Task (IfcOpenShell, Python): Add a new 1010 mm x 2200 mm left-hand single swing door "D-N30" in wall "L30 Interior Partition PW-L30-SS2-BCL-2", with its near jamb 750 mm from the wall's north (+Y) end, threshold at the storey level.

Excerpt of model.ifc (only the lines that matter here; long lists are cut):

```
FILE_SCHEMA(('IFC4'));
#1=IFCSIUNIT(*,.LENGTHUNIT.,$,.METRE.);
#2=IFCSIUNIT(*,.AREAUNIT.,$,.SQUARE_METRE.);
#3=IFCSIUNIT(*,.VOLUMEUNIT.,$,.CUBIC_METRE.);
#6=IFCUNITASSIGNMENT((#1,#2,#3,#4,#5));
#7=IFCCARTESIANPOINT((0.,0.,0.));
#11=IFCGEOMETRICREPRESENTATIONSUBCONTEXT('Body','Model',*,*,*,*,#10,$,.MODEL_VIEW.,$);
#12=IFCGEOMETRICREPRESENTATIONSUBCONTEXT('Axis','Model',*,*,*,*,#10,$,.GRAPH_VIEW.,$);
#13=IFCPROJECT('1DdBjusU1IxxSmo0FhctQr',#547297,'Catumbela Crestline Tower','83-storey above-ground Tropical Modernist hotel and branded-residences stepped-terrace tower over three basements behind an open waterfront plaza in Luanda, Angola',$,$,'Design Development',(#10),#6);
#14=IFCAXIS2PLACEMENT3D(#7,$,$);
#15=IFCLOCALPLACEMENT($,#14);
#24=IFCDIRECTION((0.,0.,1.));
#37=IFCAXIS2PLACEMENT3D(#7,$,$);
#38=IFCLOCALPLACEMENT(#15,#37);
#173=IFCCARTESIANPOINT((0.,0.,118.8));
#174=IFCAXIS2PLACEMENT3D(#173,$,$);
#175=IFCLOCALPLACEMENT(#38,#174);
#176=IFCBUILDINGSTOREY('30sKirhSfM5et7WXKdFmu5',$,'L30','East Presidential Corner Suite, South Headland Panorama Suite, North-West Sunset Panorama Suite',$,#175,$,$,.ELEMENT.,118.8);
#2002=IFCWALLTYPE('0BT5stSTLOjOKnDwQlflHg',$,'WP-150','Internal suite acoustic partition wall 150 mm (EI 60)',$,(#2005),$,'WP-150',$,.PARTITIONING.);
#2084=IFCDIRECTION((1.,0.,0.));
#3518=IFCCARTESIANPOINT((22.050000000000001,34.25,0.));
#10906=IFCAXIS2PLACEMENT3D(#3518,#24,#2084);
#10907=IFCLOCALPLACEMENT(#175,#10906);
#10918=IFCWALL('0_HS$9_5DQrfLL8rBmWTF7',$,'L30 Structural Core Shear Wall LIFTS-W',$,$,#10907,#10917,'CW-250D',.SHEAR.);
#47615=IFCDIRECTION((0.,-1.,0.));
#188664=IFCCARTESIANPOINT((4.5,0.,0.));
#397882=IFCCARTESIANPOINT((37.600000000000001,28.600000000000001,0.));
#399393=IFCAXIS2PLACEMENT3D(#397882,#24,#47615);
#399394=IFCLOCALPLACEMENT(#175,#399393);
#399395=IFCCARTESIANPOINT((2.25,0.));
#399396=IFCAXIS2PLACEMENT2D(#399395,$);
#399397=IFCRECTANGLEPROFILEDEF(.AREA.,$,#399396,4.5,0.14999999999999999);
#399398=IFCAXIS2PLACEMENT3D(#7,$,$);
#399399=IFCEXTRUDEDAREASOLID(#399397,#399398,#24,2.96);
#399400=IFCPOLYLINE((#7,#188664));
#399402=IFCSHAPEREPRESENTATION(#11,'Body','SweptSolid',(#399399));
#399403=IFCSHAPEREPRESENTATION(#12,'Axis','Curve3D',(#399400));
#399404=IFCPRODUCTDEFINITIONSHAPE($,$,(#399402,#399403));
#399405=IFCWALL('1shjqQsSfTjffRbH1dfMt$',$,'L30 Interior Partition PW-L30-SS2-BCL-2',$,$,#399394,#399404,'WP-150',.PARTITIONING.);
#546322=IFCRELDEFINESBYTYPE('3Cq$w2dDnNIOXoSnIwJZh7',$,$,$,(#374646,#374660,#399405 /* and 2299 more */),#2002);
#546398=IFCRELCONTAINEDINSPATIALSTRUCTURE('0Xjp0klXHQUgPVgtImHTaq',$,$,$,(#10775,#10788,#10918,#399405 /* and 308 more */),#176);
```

```python
import numpy as np
import ifcopenshell
import ifcopenshell.api.feature
import ifcopenshell.api.geometry
import ifcopenshell.api.root
import ifcopenshell.api.spatial
import ifcopenshell.geom
import ifcopenshell.util.element
import ifcopenshell.util.placement
import ifcopenshell.util.representation
import ifcopenshell.util.shape
import ifcopenshell.util.unit

model = ifcopenshell.open("model.ifc")
unit_scale = ifcopenshell.util.unit.calculate_unit_scale(model)
settings = ifcopenshell.geom.settings()


def volume(element):
    """Net volume in cubic metres, openings subtracted."""
    shape = ifcopenshell.geom.create_shape(settings, element)
    return ifcopenshell.util.shape.get_volume(shape.geometry)


wall = model.by_guid("1shjqQsSfTjffRbH1dfMt$")
storey = ifcopenshell.util.element.get_container(wall, ifc_class="IfcBuildingStorey")
context = ifcopenshell.util.representation.get_context(model, "Model", "Body", "MODEL_VIEW")
before = volume(wall)

width, height, from_end, sill = 1.01, 2.2, 0.75, 0.0  # metres

# The wall runs along its own X axis, and the end named is its -X end.
wall_shape = ifcopenshell.geom.create_shape(settings, wall)
x, y, z = ifcopenshell.util.shape.get_vertices(wall_shape.geometry).T
start = x.min() + from_end
face, thickness = float(y.min()), float(y.max() - y.min())
wall_matrix = ifcopenshell.util.placement.get_local_placement(wall.ObjectPlacement)
level = ifcopenshell.util.placement.get_local_placement(storey.ObjectPlacement)[2, 3]


def in_wall(x, y):
    """Placement at x, y metres in the wall's axes, at sill height."""
    matrix = wall_matrix.copy()
    matrix[:, 3] = wall_matrix @ np.array([x / unit_scale, y / unit_scale, 0.0, 1.0])
    matrix[2, 3] = level + sill / unit_scale
    return matrix


# Opening: a box that overshoots both wall faces by 50 mm.
opening = ifcopenshell.api.root.create_entity(model, ifc_class="IfcOpeningElement", predefined_type="OPENING")
box = ifcopenshell.api.geometry.add_wall_representation(
    model, context=context, length=width, height=height, thickness=thickness + 0.1
)
ifcopenshell.api.geometry.assign_representation(model, product=opening, representation=box)
ifcopenshell.api.geometry.edit_object_placement(model, product=opening, matrix=in_wall(start, face - 0.05), is_si=False)
ifcopenshell.api.feature.add_feature(model, feature=opening, element=wall)

door = ifcopenshell.api.root.create_entity(model, ifc_class="IfcDoor", name="D-N30", predefined_type="DOOR")
door.OverallWidth, door.OverallHeight = width / unit_scale, height / unit_scale
door.OperationType = "SINGLE_SWING_LEFT"
body = ifcopenshell.api.geometry.add_door_representation(
    model,
    context=context,
    overall_width=door.OverallWidth,
    overall_height=door.OverallHeight,
    operation_type="SINGLE_SWING_LEFT",
    lining_properties={"LiningDepth": thickness / unit_scale, "ThresholdDepth": thickness / unit_scale},
)
ifcopenshell.api.geometry.assign_representation(model, product=door, representation=body)
ifcopenshell.api.spatial.assign_container(model, products=[door], relating_structure=storey)
ifcopenshell.api.feature.add_filling(model, opening=opening, element=door)

# The lining spans the wall, so the door starts at the wall face.
ifcopenshell.api.geometry.edit_object_placement(model, product=door, matrix=in_wall(start, face), is_si=False)

after = volume(wall)

print(f"wall volume {before:.3f} -> {after:.3f} m3")

model.write("model-out.ifc")
```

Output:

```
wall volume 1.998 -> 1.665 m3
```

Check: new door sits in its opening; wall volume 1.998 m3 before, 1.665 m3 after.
